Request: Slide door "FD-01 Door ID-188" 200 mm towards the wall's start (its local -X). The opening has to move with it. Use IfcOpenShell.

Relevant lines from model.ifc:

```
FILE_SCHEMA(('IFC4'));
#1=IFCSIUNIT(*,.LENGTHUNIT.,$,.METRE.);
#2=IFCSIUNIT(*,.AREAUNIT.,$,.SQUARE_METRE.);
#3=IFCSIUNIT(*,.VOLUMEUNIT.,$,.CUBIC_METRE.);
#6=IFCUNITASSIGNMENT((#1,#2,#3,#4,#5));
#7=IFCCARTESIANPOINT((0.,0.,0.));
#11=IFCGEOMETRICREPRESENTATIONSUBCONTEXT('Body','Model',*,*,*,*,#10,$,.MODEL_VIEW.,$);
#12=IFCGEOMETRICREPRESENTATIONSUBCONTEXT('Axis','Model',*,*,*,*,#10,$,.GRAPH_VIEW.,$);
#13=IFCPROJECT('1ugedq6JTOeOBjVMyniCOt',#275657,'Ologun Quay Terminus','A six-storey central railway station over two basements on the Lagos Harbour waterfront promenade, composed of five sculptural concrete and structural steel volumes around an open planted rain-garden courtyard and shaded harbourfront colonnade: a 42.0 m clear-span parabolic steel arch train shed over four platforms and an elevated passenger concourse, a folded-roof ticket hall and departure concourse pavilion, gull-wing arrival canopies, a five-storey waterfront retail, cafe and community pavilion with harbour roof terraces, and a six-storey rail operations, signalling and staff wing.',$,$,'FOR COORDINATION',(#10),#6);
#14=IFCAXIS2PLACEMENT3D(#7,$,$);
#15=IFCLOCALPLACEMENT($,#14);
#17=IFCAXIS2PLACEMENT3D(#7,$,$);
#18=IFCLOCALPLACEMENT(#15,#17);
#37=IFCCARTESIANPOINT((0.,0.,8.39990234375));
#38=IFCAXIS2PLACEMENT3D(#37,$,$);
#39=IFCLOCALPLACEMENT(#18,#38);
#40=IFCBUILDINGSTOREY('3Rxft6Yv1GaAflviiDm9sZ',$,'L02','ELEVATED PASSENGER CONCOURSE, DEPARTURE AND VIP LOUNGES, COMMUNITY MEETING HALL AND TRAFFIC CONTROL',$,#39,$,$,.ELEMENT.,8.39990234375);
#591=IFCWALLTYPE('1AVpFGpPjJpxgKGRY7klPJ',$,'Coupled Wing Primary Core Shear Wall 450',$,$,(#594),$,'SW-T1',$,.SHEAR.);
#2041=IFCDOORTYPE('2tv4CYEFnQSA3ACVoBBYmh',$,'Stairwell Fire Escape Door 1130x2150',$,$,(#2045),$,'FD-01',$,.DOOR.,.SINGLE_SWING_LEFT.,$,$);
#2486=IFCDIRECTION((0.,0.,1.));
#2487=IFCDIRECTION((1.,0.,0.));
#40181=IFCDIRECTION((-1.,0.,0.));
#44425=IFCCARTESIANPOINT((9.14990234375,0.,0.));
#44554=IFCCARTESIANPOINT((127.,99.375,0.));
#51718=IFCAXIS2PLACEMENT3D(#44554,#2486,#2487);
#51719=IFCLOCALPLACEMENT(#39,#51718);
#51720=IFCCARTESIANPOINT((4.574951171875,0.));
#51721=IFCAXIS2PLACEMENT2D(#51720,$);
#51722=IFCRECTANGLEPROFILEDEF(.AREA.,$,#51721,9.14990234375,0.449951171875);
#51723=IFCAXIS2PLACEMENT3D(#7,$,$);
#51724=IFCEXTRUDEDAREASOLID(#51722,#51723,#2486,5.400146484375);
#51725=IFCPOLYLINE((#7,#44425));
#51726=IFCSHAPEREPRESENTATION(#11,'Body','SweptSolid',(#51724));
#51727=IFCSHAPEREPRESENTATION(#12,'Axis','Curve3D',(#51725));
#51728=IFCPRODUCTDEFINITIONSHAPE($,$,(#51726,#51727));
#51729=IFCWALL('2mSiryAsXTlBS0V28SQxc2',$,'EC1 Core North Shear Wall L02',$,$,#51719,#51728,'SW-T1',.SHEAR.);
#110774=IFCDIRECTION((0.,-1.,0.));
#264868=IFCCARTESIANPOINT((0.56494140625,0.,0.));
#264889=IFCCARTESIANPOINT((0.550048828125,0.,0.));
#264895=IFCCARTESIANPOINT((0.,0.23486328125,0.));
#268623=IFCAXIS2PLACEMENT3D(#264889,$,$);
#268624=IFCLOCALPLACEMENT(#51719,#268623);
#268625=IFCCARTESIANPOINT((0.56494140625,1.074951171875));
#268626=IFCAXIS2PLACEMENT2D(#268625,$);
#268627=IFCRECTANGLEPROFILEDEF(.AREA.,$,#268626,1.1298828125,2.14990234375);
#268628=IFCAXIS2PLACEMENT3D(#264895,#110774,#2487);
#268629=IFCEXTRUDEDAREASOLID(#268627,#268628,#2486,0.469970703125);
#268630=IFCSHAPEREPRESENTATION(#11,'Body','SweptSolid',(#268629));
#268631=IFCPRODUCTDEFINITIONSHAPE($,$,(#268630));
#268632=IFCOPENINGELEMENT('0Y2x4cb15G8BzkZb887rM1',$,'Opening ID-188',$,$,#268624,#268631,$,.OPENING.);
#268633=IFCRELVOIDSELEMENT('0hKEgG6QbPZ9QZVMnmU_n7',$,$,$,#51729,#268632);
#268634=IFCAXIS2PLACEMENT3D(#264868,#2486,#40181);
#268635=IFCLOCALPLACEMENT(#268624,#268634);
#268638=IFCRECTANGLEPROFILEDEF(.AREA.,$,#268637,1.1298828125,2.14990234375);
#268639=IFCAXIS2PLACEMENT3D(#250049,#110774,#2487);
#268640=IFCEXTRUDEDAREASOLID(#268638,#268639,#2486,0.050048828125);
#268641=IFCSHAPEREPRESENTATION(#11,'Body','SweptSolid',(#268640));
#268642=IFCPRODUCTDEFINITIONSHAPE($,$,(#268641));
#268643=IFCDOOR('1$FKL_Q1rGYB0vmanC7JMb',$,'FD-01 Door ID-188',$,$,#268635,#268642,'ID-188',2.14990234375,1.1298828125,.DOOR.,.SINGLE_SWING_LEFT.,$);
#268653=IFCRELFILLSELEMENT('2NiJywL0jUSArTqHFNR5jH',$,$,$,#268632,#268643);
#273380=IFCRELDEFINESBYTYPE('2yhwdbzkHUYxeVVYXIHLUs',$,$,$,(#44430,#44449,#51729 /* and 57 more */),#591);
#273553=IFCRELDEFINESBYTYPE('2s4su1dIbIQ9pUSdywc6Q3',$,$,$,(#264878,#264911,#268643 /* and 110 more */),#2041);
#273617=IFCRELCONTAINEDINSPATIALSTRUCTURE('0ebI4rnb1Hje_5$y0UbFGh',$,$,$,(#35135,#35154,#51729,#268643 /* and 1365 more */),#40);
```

```python
import ifcopenshell
import ifcopenshell.api.geometry
import ifcopenshell.util.placement

model = ifcopenshell.open("model.ifc")

door = model.by_id(268643)
opening = door.FillsVoids[0].RelatingOpeningElement
wall = opening.VoidsElements[0].RelatingBuildingElement

wall_matrix = ifcopenshell.util.placement.get_local_placement(wall.ObjectPlacement)
shift = wall_matrix[:3, 0] * -0.2
before = ifcopenshell.util.placement.get_local_placement(door.ObjectPlacement)[:3, 3].copy()

# The door is placed relative to its opening, so it follows when the opening moves.
matrix = ifcopenshell.util.placement.get_local_placement(opening.ObjectPlacement)
matrix[:3, 3] += shift
ifcopenshell.api.geometry.edit_object_placement(
    model, product=opening, matrix=matrix, is_si=False, should_transform_children=True
)

after = ifcopenshell.util.placement.get_local_placement(door.ObjectPlacement)[:3, 3]
print("door moved by", (after - before).round(3) + 0.0)

model.write("model_v2.ifc")
```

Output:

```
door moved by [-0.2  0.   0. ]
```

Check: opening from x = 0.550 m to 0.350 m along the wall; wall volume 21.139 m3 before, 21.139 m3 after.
